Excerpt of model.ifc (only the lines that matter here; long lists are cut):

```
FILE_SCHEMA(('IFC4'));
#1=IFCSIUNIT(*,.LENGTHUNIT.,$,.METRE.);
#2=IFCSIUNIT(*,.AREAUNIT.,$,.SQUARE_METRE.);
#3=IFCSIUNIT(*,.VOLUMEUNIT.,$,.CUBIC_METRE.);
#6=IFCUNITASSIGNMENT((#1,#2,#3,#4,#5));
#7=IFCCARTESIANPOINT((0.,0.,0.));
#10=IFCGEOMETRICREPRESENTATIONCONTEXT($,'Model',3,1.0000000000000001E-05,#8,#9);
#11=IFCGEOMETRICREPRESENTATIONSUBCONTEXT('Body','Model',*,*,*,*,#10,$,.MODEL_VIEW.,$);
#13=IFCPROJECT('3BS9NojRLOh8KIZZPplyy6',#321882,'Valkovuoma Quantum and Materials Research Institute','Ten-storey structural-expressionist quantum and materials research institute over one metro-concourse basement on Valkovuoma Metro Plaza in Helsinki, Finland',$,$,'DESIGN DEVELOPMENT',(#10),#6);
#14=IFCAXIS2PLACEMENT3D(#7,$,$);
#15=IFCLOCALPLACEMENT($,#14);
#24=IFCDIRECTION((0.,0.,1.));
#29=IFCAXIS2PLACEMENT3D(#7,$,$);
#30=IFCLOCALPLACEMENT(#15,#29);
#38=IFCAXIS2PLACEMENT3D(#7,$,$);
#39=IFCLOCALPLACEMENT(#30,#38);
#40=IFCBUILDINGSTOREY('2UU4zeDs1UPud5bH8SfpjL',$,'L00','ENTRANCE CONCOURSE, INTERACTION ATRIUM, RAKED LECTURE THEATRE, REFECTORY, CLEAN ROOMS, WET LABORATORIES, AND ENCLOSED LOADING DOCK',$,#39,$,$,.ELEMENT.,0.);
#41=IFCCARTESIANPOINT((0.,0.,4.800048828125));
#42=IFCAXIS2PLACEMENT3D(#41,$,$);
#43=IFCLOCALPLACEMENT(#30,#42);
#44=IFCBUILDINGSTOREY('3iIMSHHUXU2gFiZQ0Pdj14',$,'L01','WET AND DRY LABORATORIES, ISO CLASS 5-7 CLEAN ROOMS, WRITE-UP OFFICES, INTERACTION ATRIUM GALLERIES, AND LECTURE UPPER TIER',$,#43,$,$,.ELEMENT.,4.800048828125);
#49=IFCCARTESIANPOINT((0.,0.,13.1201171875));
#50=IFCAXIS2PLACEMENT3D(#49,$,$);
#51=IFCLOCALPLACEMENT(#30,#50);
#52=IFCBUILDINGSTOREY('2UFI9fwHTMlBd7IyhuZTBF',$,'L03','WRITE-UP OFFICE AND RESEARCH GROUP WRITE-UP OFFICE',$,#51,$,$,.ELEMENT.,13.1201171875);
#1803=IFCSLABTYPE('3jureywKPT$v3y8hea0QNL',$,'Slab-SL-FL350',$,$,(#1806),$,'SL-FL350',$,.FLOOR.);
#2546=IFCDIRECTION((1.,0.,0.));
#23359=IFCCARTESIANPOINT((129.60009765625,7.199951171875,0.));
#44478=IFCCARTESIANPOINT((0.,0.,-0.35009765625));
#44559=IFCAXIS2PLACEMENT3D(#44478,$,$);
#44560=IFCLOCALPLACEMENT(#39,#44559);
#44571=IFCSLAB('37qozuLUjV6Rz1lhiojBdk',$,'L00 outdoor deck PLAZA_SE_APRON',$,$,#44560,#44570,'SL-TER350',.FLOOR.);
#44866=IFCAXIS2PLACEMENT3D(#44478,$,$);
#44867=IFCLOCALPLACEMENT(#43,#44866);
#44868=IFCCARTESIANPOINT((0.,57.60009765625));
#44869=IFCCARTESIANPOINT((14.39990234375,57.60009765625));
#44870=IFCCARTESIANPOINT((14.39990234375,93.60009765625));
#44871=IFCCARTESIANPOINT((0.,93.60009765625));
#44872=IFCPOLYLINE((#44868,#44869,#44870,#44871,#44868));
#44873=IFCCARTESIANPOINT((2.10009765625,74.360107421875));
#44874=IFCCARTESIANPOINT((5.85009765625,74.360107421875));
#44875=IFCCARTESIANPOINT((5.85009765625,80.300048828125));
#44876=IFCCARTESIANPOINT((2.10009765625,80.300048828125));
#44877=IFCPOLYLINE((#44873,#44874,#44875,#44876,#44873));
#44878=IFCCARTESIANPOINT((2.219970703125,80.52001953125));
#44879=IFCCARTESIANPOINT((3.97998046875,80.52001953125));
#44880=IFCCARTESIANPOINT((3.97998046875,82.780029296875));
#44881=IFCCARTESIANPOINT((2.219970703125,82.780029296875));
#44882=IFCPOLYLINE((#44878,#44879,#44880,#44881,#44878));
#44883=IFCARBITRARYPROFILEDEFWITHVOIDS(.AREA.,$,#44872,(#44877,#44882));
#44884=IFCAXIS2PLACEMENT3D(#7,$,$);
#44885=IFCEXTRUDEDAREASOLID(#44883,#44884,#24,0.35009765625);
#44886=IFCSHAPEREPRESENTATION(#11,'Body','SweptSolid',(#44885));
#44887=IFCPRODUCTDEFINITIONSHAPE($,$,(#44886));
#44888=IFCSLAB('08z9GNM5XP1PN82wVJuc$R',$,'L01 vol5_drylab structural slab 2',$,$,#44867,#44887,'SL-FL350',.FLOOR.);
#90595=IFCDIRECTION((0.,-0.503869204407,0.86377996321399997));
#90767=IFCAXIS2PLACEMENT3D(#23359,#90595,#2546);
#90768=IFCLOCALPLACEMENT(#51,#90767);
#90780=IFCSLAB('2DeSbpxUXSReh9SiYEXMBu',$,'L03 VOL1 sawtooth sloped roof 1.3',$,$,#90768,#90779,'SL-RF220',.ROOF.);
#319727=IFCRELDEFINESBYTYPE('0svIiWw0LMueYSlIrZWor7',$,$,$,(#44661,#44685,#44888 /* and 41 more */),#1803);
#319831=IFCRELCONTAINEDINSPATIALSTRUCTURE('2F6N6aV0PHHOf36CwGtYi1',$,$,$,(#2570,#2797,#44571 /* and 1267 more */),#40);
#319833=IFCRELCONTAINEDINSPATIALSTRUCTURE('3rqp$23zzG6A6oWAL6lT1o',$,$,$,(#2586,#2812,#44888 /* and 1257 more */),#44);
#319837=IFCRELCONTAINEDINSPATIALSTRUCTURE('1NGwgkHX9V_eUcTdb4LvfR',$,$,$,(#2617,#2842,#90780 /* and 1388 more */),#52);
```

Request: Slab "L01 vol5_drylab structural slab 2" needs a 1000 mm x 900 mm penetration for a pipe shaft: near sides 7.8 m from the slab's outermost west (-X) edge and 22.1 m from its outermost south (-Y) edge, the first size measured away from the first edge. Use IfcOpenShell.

```python
import numpy as np
import ifcopenshell
import ifcopenshell.api.feature
import ifcopenshell.api.geometry
import ifcopenshell.api.root
import ifcopenshell.geom
import ifcopenshell.util.placement
import ifcopenshell.util.representation
import ifcopenshell.util.shape
import ifcopenshell.util.unit

model = ifcopenshell.open("model.ifc")
unit_scale = ifcopenshell.util.unit.calculate_unit_scale(model)
settings = ifcopenshell.geom.settings()


def volume(element):
    """Net volume in cubic metres, openings subtracted."""
    shape = ifcopenshell.geom.create_shape(settings, element)
    return ifcopenshell.util.shape.get_volume(shape.geometry)


slab = model.by_id(44888)
before = volume(slab)

# Extent in the slab's own axes, in metres. The edges named are its -X and -Y sides.
slab_shape = ifcopenshell.geom.create_shape(settings, slab)
vertices = ifcopenshell.util.shape.get_vertices(slab_shape.geometry)
x_min, y_min, bottom = vertices.min(axis=0)
top = vertices[:, 2].max()

opening = ifcopenshell.api.root.create_entity(model, ifc_class="IfcOpeningElement", name="Pipe shaft opening", predefined_type="OPENING")
context = ifcopenshell.util.representation.get_context(model, "Model", "Body", "MODEL_VIEW")
width, depth = 1, 0.9
outline = [(0.0, 0.0), (width, 0.0), (width, depth), (0.0, depth), (0.0, 0.0)]
# Overshoot both faces by 50 mm so the cut is clean.
shape = ifcopenshell.api.geometry.add_slab_representation(
    model, context=context, depth=top - bottom + 0.1, polyline=outline
)
ifcopenshell.api.geometry.assign_representation(model, product=opening, representation=shape)

matrix = ifcopenshell.util.placement.get_local_placement(slab.ObjectPlacement)
matrix[:, 3] = matrix @ np.append(np.array([x_min + 7.8, y_min + 22.1, bottom - 0.05]) / unit_scale, 1.0)
ifcopenshell.api.geometry.edit_object_placement(model, product=opening, matrix=matrix, is_si=False)
ifcopenshell.api.feature.add_feature(model, feature=opening, element=slab)

after = volume(slab)

print(f"slab volume {before:.3f} -> {after:.3f} m3")

model.write("model_rev.ifc")
```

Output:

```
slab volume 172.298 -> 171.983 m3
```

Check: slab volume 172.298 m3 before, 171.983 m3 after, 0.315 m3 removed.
